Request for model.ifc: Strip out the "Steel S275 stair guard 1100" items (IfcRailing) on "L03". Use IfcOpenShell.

First a look at what the model holds.

```python
import ifcopenshell
import ifcopenshell.util.element

model = ifcopenshell.open("model.ifc")
print(model.schema)
storey = next(s for s in model.by_type("IfcBuildingStorey") if s.Name == "L03")
railings = [e for e in ifcopenshell.util.element.get_decomposition(storey) if e.is_a("IfcRailing")]
seen = {}
for e in railings:
    element_type = ifcopenshell.util.element.get_type(e)
    name = element_type.Name if element_type not in (None, e) else None
    seen[name] = seen.get(name, 0) + 1
for name, count in sorted(seen.items(), key=str):
    print(count, "x", name)
```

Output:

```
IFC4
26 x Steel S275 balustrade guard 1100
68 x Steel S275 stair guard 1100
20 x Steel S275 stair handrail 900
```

```python
import ifcopenshell
import ifcopenshell.api.root
import ifcopenshell.util.element

model = ifcopenshell.open("model.ifc")

storey = next(s for s in model.by_type("IfcBuildingStorey") if s.Name == "L03")
railings = [e for e in ifcopenshell.util.element.get_decomposition(storey) if e.is_a("IfcRailing")]
targets = [e for e in railings if (t := ifcopenshell.util.element.get_type(e)) not in (None, e) and t.Name == "Steel S275 stair guard 1100"]

for e in targets:
    ifcopenshell.api.root.remove_product(model, product=e)
print(len(targets), "removed")

model.write("model_rev.ifc")
```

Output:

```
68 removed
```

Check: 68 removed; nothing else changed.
